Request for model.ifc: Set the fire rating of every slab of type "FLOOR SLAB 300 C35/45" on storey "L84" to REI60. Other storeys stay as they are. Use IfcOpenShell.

First a look at what the model holds.

```python
import ifcopenshell
import ifcopenshell.util.element

model = ifcopenshell.open("model.ifc")
print(model.schema)
storey = next(s for s in model.by_type("IfcBuildingStorey") if s.Name == "L84")
slabs = [e for e in ifcopenshell.util.element.get_decomposition(storey) if e.is_a("IfcSlab")]
seen = {}
for e in slabs:
    element_type = ifcopenshell.util.element.get_type(e)
    key = (element_type.Name if element_type != e and element_type else None, ifcopenshell.util.element.get_pset(e, "Pset_SlabCommon", "FireRating"))
    seen[key] = seen.get(key, 0) + 1
for (name, value), count in sorted(seen.items(), key=str):
    print(count, "x", name, "|", value)
```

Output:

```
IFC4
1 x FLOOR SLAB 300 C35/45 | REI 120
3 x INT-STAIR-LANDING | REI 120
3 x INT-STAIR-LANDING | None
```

```python
import ifcopenshell
import ifcopenshell.api.pset
import ifcopenshell.util.element

model = ifcopenshell.open("model.ifc")

storey = next(s for s in model.by_type("IfcBuildingStorey") if s.Name == "L84")
slabs = [e for e in ifcopenshell.util.element.get_decomposition(storey) if e.is_a("IfcSlab")]

count = 0
for e in slabs:
    element_type = ifcopenshell.util.element.get_type(e)
    if element_type in (None, e) or element_type.Name != "FLOOR SLAB 300 C35/45":
        continue
    found = ifcopenshell.util.element.get_pset(e, "Pset_SlabCommon", should_inherit=False)
    if found:
        pset = model.by_id(found["id"])
        if len(ifcopenshell.util.element.get_elements_by_pset(pset)) > 1:
            pset = ifcopenshell.api.pset.unshare_pset(model, products=[e], pset=pset)[0]
    else:
        pset = ifcopenshell.api.pset.add_pset(model, product=e, name="Pset_SlabCommon")
    ifcopenshell.api.pset.edit_pset(model, pset=pset, properties={"FireRating": "REI60"})
    count += 1

print(count, "slabs updated")

model.write("model-out.ifc")
```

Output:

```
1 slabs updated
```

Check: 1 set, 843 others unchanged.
